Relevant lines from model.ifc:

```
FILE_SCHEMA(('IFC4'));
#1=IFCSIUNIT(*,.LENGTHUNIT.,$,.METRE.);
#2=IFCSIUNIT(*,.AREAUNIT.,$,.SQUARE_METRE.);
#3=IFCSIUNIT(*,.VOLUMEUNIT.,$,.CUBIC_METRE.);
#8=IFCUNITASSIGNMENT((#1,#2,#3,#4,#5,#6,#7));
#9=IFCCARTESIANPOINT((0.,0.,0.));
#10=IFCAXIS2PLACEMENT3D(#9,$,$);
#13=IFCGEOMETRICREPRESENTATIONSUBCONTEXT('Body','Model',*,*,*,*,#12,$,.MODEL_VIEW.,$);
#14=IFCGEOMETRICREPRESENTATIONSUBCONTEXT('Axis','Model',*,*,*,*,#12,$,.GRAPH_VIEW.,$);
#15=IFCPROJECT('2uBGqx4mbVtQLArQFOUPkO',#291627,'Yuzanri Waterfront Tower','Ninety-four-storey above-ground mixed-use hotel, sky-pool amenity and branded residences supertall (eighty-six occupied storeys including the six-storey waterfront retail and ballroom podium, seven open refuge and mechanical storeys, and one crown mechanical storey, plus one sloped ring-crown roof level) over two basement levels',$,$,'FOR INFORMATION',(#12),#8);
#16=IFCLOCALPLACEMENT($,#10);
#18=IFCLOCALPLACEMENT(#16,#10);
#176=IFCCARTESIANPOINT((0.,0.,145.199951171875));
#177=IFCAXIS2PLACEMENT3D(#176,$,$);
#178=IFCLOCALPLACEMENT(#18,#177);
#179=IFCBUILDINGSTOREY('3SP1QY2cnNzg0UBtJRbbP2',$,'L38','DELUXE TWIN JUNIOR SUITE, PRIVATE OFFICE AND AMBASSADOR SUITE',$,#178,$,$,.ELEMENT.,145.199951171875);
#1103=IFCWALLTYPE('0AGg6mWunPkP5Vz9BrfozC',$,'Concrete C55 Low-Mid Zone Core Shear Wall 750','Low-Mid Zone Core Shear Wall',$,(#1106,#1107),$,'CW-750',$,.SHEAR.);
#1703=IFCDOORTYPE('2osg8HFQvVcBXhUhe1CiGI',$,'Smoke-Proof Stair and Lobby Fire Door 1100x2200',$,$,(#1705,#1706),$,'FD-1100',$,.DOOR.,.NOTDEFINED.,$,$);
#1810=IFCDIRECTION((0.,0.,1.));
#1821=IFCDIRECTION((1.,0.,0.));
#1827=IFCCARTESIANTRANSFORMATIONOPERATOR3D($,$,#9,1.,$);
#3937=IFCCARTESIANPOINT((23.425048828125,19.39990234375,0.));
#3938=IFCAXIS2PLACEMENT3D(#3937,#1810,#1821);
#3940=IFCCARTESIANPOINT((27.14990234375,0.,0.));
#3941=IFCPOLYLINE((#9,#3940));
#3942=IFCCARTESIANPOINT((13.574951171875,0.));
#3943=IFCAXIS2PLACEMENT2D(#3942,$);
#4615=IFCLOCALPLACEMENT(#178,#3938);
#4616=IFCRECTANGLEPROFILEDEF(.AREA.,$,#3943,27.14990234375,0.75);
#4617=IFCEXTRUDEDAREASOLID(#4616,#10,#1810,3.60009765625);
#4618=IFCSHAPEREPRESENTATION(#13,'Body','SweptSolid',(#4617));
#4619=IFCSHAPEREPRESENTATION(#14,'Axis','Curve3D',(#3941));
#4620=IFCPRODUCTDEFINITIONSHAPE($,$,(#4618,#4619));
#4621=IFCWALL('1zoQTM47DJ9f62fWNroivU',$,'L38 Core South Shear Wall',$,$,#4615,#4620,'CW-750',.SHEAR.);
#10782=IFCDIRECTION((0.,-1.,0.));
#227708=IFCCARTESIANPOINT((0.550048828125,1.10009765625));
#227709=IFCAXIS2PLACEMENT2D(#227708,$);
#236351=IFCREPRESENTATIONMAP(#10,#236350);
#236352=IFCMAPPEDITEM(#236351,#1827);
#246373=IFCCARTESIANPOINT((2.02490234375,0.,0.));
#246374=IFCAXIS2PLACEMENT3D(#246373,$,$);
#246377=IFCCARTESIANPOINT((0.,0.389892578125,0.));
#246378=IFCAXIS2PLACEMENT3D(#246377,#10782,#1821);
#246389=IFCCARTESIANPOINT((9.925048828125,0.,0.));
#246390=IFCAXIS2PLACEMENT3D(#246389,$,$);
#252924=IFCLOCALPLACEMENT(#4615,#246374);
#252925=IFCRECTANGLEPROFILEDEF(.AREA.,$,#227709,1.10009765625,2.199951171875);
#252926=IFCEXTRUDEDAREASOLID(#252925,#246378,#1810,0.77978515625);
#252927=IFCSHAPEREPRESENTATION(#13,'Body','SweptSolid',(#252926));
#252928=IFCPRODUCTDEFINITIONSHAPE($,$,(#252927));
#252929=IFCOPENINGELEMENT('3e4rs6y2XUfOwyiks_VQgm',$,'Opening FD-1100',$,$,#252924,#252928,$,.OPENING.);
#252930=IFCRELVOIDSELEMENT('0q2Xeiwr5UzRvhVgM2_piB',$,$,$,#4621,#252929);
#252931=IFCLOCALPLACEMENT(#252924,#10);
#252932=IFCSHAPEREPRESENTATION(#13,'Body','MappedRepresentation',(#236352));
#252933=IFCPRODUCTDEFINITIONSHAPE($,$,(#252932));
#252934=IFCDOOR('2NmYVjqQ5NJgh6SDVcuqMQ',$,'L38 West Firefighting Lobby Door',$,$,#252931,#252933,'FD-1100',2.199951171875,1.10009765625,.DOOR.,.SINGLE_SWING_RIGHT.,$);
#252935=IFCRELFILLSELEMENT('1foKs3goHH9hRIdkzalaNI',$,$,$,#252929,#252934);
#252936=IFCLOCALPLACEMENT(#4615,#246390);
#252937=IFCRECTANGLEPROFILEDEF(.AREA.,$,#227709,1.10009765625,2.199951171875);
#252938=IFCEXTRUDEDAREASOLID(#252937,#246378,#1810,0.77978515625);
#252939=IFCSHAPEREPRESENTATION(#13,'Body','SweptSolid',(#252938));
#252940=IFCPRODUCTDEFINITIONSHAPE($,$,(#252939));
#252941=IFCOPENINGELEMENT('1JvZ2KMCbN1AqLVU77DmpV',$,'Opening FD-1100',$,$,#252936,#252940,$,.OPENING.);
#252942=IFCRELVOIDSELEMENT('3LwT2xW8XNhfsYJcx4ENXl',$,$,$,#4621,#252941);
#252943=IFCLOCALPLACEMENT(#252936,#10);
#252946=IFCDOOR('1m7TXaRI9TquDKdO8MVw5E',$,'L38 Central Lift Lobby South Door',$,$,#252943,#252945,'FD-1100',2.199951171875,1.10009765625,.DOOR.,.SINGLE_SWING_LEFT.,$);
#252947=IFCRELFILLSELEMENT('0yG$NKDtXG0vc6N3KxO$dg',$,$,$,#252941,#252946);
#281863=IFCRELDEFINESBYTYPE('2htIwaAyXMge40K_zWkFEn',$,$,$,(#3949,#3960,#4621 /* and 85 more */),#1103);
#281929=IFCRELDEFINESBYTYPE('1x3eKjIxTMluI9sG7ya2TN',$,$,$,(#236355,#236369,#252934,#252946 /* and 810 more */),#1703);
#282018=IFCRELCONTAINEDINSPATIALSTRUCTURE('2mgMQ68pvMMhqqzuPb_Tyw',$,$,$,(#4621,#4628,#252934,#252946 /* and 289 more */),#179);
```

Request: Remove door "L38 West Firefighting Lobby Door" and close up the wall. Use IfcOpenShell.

```python
import ifcopenshell
import ifcopenshell.api.feature
import ifcopenshell.api.root
import ifcopenshell.geom
import ifcopenshell.util.shape

model = ifcopenshell.open("model.ifc")
settings = ifcopenshell.geom.settings()


def volume(element):
    """Net volume in cubic metres, openings subtracted."""
    shape = ifcopenshell.geom.create_shape(settings, element)
    return ifcopenshell.util.shape.get_volume(shape.geometry)


door = model.by_guid("2NmYVjqQ5NJgh6SDVcuqMQ")
opening = door.FillsVoids[0].RelatingOpeningElement
wall = opening.VoidsElements[0].RelatingBuildingElement
before = volume(wall)

ifcopenshell.api.root.remove_product(model, product=door)
ifcopenshell.api.feature.remove_feature(model, feature=opening)

after = volume(wall)

print(f"wall volume {before:.3f} -> {after:.3f} m3")

model.write("model_updated.ifc")
```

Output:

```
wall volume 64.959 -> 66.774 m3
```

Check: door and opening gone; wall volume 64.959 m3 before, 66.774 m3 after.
